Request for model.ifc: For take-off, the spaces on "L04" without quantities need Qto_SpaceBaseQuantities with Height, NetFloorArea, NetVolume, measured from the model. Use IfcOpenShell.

First a look at what the model holds.

```python
import ifcopenshell
import ifcopenshell.util.element
import ifcopenshell.util.unit

model = ifcopenshell.open("model.ifc")
print(model.schema)
for unit_type in ("LENGTHUNIT", "AREAUNIT", "VOLUMEUNIT"):
    print(unit_type, ifcopenshell.util.unit.calculate_unit_scale(model, unit_type))
storey = next(s for s in model.by_type("IfcBuildingStorey") if s.Name == "L04")
spaces = [e for e in ifcopenshell.util.element.get_decomposition(storey) if e.is_a("IfcSpace")]
for e in sorted(spaces, key=lambda e: e.id()):
    print(e.id(), e.is_a(), e.Name, list(ifcopenshell.util.element.get_psets(e, qtos_only=True)), sep=" | ")
```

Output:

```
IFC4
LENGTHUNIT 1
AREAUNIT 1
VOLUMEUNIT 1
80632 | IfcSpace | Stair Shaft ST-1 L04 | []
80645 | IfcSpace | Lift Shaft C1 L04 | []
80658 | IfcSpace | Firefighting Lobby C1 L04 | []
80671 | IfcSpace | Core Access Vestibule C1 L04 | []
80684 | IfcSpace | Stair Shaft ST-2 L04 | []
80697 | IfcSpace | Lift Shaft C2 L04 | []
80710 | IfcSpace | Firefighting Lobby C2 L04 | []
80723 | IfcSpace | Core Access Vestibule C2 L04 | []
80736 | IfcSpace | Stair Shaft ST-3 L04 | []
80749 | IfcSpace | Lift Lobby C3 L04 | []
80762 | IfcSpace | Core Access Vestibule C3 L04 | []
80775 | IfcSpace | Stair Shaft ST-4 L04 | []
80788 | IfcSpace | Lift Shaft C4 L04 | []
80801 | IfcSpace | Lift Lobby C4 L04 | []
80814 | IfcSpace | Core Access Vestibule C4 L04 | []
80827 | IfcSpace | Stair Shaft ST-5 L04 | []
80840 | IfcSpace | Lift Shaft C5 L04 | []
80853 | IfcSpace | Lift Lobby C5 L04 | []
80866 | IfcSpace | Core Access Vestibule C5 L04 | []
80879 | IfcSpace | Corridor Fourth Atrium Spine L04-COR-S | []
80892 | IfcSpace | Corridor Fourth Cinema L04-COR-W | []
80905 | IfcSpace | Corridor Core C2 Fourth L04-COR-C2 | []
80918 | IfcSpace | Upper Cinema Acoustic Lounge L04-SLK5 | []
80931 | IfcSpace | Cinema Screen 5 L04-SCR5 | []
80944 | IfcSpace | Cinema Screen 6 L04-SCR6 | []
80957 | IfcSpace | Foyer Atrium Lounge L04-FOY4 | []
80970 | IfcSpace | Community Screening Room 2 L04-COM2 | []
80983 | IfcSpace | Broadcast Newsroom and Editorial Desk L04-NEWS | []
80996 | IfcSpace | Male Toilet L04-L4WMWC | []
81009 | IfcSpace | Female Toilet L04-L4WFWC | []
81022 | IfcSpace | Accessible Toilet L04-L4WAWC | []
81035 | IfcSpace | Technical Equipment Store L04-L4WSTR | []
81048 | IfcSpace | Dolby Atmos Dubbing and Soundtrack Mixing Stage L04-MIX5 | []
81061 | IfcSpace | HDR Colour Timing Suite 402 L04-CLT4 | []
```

```python
import ifcopenshell
import ifcopenshell.api.pset
import ifcopenshell.geom
import ifcopenshell.util.element
import ifcopenshell.util.shape
import ifcopenshell.util.unit

model = ifcopenshell.open("model.ifc")
unit_scale = ifcopenshell.util.unit.calculate_unit_scale(model)
area_scale = ifcopenshell.util.unit.calculate_unit_scale(model, "AREAUNIT")
volume_scale = ifcopenshell.util.unit.calculate_unit_scale(model, "VOLUMEUNIT")
settings = ifcopenshell.geom.settings()

storey = next(s for s in model.by_type("IfcBuildingStorey") if s.Name == "L04")
spaces = [e for e in ifcopenshell.util.element.get_decomposition(storey) if e.is_a("IfcSpace")]

for e in sorted(spaces, key=lambda e: e.id()):
    if ifcopenshell.util.element.get_psets(e, qtos_only=True, should_inherit=False):
        continue
    # Geometry comes back in metres, in the element's own axes.
    shape = ifcopenshell.geom.create_shape(settings, e)
    values = {
        "Height": ifcopenshell.util.shape.get_z(shape.geometry) / unit_scale,
        "NetFloorArea": ifcopenshell.util.shape.get_footprint_area(shape.geometry) / area_scale,
        "NetVolume": ifcopenshell.util.shape.get_volume(shape.geometry) / volume_scale,
    }
    qto = ifcopenshell.api.pset.add_qto(model, product=e, name="Qto_SpaceBaseQuantities")
    ifcopenshell.api.pset.edit_qto(model, qto=qto, properties=values)
    print(e.id(), {k: round(v, 3) for k, v in values.items()})

model.write("model_updated.ifc")
```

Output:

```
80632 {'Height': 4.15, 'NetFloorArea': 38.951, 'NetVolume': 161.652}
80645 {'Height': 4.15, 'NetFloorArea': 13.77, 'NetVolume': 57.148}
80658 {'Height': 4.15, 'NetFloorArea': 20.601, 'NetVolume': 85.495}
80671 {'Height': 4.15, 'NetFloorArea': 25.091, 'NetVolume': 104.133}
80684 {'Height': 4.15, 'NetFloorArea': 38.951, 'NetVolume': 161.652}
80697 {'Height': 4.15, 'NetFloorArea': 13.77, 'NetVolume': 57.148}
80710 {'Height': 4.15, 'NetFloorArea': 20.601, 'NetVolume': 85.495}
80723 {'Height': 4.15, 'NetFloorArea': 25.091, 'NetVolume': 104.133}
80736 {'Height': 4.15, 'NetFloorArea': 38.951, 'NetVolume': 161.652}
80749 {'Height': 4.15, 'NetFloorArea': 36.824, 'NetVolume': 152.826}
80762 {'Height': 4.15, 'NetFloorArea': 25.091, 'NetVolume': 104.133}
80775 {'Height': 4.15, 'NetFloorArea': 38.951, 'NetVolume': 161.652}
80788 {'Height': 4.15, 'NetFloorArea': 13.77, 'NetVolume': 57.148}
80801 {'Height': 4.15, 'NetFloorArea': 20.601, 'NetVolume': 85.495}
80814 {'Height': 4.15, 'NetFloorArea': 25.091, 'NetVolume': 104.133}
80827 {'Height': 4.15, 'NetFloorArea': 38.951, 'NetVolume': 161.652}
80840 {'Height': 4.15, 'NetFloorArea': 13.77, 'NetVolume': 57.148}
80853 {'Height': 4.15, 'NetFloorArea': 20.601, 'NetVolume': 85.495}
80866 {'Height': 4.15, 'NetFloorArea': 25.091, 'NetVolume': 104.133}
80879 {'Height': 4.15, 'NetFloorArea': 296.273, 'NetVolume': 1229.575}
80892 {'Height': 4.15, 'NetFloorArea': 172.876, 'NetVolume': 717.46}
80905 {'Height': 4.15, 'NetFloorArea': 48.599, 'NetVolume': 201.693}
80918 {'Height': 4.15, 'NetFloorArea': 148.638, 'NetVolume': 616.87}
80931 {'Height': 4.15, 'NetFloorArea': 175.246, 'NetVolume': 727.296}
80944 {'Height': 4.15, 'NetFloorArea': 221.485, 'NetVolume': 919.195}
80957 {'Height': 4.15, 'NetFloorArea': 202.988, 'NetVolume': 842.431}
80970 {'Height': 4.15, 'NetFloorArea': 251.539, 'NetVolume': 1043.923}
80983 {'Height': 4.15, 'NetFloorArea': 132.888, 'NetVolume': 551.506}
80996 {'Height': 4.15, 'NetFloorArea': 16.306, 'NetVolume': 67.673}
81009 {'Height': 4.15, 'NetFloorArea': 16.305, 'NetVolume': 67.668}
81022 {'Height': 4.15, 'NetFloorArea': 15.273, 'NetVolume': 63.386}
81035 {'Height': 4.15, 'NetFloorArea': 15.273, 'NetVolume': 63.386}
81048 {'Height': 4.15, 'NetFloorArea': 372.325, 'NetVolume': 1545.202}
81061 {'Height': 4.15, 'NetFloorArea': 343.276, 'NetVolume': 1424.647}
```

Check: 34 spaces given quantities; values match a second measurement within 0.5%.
